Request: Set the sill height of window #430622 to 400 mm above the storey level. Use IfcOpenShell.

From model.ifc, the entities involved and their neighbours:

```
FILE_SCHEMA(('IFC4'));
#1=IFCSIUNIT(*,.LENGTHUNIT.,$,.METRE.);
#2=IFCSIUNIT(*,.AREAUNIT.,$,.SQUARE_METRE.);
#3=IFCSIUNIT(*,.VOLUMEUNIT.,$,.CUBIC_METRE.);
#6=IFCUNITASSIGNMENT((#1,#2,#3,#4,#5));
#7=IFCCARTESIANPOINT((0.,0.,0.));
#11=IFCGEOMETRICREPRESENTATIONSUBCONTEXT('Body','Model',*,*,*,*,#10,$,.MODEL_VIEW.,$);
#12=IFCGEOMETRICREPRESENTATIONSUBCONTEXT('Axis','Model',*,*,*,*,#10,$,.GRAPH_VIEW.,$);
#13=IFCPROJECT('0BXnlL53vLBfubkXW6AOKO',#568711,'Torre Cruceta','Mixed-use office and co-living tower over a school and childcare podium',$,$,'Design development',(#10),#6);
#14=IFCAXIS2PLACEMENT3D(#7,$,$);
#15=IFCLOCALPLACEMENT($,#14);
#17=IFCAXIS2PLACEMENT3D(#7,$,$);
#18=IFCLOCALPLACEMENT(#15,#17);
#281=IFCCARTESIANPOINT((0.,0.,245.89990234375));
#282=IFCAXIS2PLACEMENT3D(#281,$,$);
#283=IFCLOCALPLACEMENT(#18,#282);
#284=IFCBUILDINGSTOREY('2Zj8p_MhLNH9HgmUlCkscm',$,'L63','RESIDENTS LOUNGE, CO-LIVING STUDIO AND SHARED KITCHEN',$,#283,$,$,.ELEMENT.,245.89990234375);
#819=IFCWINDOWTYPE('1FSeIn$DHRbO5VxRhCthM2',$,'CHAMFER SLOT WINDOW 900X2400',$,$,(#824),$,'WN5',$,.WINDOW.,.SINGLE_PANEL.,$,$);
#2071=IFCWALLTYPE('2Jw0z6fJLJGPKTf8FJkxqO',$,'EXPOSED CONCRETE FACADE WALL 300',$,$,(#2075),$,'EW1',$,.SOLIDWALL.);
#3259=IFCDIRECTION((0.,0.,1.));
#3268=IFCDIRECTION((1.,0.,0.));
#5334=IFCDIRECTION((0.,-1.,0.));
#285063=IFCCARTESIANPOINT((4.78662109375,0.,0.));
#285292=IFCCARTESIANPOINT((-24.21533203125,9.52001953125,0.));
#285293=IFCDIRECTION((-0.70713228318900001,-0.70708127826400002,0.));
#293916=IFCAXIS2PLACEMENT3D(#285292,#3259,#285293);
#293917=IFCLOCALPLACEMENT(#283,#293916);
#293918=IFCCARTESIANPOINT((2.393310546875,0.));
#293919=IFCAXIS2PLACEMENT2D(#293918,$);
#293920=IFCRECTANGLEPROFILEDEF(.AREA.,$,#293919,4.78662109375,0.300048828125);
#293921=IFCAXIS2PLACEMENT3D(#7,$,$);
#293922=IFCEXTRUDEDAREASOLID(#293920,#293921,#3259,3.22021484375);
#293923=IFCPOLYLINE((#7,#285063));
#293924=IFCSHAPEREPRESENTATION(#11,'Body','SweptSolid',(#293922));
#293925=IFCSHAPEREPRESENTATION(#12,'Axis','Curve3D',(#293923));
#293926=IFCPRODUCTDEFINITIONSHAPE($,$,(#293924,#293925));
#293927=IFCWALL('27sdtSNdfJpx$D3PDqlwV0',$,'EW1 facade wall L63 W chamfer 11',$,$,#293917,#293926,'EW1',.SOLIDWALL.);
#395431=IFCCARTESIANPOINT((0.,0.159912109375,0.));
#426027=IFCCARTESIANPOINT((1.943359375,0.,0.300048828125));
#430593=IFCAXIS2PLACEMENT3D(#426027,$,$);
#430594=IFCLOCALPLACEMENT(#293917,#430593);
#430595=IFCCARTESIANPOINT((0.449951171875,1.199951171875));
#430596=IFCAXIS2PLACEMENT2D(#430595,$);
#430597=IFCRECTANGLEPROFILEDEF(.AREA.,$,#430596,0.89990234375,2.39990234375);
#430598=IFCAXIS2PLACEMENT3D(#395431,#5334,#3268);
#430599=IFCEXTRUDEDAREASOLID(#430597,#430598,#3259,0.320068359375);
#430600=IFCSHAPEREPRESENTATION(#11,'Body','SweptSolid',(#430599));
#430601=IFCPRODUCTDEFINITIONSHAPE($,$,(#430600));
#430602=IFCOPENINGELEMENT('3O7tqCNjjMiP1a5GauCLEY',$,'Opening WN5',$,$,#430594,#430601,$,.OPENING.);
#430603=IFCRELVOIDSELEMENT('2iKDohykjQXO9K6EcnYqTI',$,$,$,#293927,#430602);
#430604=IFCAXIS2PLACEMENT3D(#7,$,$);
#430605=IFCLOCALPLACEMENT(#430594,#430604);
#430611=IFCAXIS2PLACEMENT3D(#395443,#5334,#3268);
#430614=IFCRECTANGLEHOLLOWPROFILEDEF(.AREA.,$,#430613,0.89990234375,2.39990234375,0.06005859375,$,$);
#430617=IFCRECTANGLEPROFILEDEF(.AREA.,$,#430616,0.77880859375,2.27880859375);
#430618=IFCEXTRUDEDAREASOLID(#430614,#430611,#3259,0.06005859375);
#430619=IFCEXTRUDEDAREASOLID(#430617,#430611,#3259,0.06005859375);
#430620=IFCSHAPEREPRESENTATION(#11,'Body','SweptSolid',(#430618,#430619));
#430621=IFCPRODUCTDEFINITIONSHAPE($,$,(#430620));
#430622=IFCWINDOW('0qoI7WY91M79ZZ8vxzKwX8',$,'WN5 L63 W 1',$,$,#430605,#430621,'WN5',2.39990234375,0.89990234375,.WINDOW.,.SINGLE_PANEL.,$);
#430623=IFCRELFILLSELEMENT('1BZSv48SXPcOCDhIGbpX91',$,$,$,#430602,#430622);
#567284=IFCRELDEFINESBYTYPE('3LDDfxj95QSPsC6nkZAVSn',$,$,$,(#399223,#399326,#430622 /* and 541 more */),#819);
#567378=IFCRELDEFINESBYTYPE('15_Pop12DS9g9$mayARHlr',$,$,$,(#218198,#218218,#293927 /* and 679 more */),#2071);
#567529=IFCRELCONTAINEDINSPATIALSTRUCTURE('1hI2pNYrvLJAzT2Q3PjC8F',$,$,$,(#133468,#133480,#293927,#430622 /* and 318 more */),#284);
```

```python
import numpy as np
import ifcopenshell
import ifcopenshell.api.geometry
import ifcopenshell.geom
import ifcopenshell.util.element
import ifcopenshell.util.placement
import ifcopenshell.util.shape
import ifcopenshell.util.unit

model = ifcopenshell.open("model.ifc")
unit_scale = ifcopenshell.util.unit.calculate_unit_scale(model)

window = model.by_guid("0qoI7WY91M79ZZ8vxzKwX8")
opening = window.FillsVoids[0].RelatingOpeningElement
storey = ifcopenshell.util.element.get_container(window, ifc_class="IfcBuildingStorey")
level = ifcopenshell.util.placement.get_local_placement(storey.ObjectPlacement)[2, 3]

# The opening's origin need not be at the sill, so measure its lowest point.
shape = ifcopenshell.geom.create_shape(ifcopenshell.geom.settings(), opening)
bottom = ifcopenshell.util.shape.get_shape_bottom_elevation(shape, shape.geometry) / unit_scale
dz = level + 0.4 - bottom

shift = np.array([0.0, 0.0, dz])
# The window is placed relative to its opening, so it follows when the opening moves.
matrix = ifcopenshell.util.placement.get_local_placement(opening.ObjectPlacement)
matrix[:3, 3] += shift
ifcopenshell.api.geometry.edit_object_placement(
    model, product=opening, matrix=matrix, is_si=False, should_transform_children=True
)

print(f"moved by {dz * unit_scale:+.3f} m")

model.write("model-out.ifc")
```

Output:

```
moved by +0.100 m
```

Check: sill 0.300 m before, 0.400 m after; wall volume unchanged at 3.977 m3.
